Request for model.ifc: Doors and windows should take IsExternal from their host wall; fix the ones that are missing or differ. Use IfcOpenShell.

First a look at what the model holds.

```python
import ifcopenshell
import ifcopenshell.util.element

model = ifcopenshell.open("model.ifc")
print(model.schema)
seen = {}
for e in model.by_type("IfcDoor") + model.by_type("IfcWindow"):
    if not e.FillsVoids:
        continue
    host = e.FillsVoids[0].RelatingOpeningElement.VoidsElements[0].RelatingBuildingElement
    own = ifcopenshell.util.element.get_pset(e, f"Pset_{e.is_a()[3:].removesuffix('StandardCase')}Common", "IsExternal")
    wall = ifcopenshell.util.element.get_pset(host, "Pset_WallCommon", "IsExternal")
    seen[e.is_a(), own, wall] = seen.get((e.is_a(), own, wall), 0) + 1
for (cls, own, wall), count in sorted(seen.items(), key=str):
    print(count, cls, "IsExternal:", own, "| host wall:", wall)
```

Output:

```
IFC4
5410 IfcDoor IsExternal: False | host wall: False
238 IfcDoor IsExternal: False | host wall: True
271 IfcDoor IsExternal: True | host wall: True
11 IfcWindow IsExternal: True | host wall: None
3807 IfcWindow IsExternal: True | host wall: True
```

```python
import ifcopenshell
import ifcopenshell.api.pset
import ifcopenshell.util.element

model = ifcopenshell.open("model.ifc")

count = 0
for ifc_class, pset_name in (("IfcDoor", "Pset_DoorCommon"), ("IfcWindow", "Pset_WindowCommon")):
    for e in model.by_type(ifc_class):
        if not e.FillsVoids:
            continue
        host = e.FillsVoids[0].RelatingOpeningElement.VoidsElements[0].RelatingBuildingElement
        external = ifcopenshell.util.element.get_pset(host, "Pset_WallCommon", "IsExternal")
        if external is None or ifcopenshell.util.element.get_pset(e, pset_name, "IsExternal") == external:
            continue
        pset = ifcopenshell.api.pset.add_pset(model, product=e, name=pset_name)
        ifcopenshell.api.pset.edit_pset(model, pset=pset, properties={"IsExternal": external})
        count += 1

print(count, "updated")

model.write("model_rev.ifc")
```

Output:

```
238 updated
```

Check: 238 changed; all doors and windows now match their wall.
